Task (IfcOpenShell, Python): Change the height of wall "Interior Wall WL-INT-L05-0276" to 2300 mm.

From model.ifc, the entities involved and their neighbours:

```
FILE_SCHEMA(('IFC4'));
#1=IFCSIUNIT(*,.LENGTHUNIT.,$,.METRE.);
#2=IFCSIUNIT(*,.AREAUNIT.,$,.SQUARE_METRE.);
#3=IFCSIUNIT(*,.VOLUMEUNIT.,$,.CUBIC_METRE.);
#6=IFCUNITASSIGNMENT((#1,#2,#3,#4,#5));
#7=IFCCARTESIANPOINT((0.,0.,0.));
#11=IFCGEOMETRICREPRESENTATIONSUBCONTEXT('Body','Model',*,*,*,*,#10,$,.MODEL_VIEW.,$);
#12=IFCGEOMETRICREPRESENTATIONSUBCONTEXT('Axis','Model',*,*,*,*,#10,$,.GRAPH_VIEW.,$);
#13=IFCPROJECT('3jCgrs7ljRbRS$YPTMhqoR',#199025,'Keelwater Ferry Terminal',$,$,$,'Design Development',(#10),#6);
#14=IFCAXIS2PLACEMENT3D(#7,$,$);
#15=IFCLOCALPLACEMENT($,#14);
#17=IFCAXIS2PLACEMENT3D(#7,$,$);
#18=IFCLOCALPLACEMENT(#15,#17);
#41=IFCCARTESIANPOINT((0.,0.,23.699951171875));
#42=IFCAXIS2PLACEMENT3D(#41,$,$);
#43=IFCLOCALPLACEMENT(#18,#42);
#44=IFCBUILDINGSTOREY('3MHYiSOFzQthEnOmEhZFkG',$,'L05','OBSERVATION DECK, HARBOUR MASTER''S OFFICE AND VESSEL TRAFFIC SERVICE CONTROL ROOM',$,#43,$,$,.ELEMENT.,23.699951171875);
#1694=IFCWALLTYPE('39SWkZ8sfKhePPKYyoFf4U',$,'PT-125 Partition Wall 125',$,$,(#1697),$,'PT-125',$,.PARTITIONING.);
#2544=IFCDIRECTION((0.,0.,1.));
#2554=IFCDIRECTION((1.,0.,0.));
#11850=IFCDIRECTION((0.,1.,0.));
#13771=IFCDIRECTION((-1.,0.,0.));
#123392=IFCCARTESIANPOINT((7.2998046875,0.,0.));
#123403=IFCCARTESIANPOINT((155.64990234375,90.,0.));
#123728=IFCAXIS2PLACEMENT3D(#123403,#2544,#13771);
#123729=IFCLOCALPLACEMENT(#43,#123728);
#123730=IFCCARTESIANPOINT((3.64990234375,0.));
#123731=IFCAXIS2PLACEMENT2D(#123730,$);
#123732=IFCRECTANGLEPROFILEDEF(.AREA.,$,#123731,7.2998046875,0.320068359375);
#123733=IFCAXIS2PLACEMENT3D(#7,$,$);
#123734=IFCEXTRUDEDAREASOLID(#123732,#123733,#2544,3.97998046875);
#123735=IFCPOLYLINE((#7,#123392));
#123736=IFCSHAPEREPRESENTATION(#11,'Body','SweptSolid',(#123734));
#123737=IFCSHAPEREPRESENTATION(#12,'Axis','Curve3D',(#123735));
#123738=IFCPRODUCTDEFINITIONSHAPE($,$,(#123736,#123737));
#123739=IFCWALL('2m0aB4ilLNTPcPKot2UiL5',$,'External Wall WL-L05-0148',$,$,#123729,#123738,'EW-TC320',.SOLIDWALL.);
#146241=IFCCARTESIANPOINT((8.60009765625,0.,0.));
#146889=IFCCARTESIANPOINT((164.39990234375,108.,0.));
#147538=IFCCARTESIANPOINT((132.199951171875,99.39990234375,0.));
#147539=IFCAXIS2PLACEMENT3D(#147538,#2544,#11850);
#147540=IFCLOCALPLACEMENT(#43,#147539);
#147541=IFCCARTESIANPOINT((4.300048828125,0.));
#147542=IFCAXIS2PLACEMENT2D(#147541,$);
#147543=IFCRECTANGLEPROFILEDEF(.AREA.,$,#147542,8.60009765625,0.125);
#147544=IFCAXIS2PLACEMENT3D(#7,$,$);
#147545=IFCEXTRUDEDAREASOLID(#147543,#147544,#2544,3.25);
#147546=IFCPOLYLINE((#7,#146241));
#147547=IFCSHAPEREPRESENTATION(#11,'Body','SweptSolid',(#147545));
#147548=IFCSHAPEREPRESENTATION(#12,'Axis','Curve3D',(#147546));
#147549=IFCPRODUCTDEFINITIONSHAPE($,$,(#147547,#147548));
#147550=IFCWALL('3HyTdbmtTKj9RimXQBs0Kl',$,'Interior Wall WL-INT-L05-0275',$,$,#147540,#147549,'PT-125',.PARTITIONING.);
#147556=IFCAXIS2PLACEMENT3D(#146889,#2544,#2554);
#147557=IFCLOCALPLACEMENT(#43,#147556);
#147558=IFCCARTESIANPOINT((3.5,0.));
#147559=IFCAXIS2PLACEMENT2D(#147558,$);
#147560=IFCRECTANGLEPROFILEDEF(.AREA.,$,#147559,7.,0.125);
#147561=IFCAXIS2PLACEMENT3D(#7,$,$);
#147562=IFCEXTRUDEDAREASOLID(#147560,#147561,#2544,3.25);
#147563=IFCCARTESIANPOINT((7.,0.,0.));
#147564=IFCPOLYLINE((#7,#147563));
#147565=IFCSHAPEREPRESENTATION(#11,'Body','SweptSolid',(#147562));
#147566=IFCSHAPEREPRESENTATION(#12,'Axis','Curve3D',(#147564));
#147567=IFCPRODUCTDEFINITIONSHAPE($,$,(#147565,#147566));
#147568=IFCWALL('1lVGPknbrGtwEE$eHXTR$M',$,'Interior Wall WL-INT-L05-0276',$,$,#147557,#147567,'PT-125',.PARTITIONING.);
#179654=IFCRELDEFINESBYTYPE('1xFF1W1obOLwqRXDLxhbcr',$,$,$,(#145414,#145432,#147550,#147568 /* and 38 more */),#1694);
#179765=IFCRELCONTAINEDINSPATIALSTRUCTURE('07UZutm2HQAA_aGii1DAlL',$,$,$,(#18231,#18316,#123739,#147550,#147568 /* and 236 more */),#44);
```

```python
import ifcopenshell
import ifcopenshell.geom
import ifcopenshell.util.representation
import ifcopenshell.util.shape

model = ifcopenshell.open("model.ifc")
settings = ifcopenshell.geom.settings()


def volume(element):
    """Net volume in cubic metres, openings subtracted."""
    shape = ifcopenshell.geom.create_shape(settings, element)
    return ifcopenshell.util.shape.get_volume(shape.geometry)


wall = model.by_guid("1lVGPknbrGtwEE$eHXTR$M")
before = volume(wall)

body = ifcopenshell.util.representation.get_representation(wall, "Model", "Body")
solid = body.Items[0]
old_height = solid.Depth
solid.Depth = 2.3
after = volume(wall)

print(f"height {old_height:g} -> {solid.Depth:g}, volume {before:.3f} -> {after:.3f} m3")

model.write("model_edited.ifc")
```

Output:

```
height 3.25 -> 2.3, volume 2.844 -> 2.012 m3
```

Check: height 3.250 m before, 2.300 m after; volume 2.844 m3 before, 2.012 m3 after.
